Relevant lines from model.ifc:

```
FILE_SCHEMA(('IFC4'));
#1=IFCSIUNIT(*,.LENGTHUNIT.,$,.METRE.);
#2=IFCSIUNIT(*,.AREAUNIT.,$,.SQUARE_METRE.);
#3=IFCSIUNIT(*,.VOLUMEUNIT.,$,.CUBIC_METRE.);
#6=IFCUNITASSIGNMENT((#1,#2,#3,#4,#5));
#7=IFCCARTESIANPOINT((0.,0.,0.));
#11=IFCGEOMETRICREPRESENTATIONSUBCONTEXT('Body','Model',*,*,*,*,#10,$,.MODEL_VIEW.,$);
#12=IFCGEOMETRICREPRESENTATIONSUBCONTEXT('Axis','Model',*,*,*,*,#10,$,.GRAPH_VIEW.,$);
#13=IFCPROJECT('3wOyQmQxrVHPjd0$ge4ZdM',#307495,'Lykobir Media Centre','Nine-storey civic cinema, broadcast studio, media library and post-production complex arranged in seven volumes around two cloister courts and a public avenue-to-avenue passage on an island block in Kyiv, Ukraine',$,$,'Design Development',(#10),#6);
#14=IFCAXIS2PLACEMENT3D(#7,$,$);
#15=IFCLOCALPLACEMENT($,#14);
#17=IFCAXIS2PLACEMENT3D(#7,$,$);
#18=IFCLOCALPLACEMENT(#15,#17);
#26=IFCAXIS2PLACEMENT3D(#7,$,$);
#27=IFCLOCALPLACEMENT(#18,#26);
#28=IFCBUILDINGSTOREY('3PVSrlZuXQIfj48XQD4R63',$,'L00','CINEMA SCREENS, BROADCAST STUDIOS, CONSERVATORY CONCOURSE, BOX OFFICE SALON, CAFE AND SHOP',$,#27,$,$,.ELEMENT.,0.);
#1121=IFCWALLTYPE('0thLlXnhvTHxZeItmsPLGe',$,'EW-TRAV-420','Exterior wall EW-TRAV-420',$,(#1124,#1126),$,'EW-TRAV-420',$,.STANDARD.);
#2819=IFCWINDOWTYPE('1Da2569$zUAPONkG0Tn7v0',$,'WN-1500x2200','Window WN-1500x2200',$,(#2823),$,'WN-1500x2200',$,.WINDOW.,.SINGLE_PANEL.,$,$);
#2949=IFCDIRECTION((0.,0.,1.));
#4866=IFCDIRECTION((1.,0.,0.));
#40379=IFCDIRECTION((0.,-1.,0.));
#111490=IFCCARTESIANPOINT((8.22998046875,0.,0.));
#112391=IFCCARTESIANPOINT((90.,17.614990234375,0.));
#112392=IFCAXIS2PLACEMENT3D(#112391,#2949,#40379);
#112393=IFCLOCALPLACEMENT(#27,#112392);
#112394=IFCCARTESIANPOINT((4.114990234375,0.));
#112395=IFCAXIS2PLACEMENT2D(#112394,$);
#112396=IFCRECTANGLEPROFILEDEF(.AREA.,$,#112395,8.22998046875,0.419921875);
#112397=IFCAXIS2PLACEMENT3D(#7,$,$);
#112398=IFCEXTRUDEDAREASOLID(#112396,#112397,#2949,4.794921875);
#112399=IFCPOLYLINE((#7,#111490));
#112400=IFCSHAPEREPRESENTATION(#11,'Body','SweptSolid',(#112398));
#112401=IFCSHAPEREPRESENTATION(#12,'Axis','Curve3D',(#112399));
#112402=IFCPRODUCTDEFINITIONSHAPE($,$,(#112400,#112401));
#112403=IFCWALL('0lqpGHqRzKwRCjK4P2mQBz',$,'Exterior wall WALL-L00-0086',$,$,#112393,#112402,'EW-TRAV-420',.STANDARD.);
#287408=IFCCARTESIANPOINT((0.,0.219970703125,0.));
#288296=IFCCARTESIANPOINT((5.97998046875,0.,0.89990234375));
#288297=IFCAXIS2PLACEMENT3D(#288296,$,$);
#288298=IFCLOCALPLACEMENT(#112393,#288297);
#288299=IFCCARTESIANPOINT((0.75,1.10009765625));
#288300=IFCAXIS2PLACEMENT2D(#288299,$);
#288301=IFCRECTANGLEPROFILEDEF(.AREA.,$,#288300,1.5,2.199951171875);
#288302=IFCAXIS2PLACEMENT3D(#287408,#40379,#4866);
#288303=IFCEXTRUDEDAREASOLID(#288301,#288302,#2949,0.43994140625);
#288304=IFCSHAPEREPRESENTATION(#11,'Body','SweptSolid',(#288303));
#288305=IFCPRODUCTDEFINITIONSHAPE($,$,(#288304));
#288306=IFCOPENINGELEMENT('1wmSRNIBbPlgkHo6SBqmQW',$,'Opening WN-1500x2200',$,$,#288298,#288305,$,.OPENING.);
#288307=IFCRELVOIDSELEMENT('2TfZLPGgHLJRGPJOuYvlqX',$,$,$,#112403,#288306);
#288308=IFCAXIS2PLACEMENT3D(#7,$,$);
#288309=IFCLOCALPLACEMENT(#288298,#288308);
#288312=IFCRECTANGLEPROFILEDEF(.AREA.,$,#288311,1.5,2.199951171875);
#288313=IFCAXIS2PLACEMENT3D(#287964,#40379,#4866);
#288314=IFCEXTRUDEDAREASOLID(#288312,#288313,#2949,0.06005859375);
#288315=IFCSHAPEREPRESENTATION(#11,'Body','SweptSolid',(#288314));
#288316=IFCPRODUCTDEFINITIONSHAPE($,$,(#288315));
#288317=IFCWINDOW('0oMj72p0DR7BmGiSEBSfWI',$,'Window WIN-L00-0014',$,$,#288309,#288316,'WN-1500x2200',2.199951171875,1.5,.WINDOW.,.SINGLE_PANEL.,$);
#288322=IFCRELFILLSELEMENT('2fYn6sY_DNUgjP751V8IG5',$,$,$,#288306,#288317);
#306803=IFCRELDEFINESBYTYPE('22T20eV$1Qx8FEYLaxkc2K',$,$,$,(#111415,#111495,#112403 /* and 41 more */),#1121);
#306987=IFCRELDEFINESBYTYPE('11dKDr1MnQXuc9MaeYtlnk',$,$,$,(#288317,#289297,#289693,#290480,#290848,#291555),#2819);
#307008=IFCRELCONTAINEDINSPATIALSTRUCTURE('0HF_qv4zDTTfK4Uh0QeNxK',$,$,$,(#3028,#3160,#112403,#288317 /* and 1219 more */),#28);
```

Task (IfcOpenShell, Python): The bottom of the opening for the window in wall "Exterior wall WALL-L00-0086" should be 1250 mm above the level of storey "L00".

```python
import numpy as np
import ifcopenshell
import ifcopenshell.api.geometry
import ifcopenshell.geom
import ifcopenshell.util.element
import ifcopenshell.util.placement
import ifcopenshell.util.shape
import ifcopenshell.util.unit

model = ifcopenshell.open("model.ifc")
unit_scale = ifcopenshell.util.unit.calculate_unit_scale(model)

window = model.by_guid("0oMj72p0DR7BmGiSEBSfWI")
opening = window.FillsVoids[0].RelatingOpeningElement
storey = ifcopenshell.util.element.get_container(window, ifc_class="IfcBuildingStorey")
level = ifcopenshell.util.placement.get_local_placement(storey.ObjectPlacement)[2, 3]

# The opening's origin need not be at the sill, so measure its lowest point.
shape = ifcopenshell.geom.create_shape(ifcopenshell.geom.settings(), opening)
bottom = ifcopenshell.util.shape.get_shape_bottom_elevation(shape, shape.geometry) / unit_scale
dz = level + 1.25 / unit_scale - bottom

shift = np.array([0.0, 0.0, dz])
# The window is placed relative to its opening, so it follows when the opening moves.
matrix = ifcopenshell.util.placement.get_local_placement(opening.ObjectPlacement)
matrix[:3, 3] += shift
ifcopenshell.api.geometry.edit_object_placement(
    model, product=opening, matrix=matrix, is_si=False, should_transform_children=True
)

print(f"moved by {dz * unit_scale:+.3f} m")

model.write("model_v2.ifc")
```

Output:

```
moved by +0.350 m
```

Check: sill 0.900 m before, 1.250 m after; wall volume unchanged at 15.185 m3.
